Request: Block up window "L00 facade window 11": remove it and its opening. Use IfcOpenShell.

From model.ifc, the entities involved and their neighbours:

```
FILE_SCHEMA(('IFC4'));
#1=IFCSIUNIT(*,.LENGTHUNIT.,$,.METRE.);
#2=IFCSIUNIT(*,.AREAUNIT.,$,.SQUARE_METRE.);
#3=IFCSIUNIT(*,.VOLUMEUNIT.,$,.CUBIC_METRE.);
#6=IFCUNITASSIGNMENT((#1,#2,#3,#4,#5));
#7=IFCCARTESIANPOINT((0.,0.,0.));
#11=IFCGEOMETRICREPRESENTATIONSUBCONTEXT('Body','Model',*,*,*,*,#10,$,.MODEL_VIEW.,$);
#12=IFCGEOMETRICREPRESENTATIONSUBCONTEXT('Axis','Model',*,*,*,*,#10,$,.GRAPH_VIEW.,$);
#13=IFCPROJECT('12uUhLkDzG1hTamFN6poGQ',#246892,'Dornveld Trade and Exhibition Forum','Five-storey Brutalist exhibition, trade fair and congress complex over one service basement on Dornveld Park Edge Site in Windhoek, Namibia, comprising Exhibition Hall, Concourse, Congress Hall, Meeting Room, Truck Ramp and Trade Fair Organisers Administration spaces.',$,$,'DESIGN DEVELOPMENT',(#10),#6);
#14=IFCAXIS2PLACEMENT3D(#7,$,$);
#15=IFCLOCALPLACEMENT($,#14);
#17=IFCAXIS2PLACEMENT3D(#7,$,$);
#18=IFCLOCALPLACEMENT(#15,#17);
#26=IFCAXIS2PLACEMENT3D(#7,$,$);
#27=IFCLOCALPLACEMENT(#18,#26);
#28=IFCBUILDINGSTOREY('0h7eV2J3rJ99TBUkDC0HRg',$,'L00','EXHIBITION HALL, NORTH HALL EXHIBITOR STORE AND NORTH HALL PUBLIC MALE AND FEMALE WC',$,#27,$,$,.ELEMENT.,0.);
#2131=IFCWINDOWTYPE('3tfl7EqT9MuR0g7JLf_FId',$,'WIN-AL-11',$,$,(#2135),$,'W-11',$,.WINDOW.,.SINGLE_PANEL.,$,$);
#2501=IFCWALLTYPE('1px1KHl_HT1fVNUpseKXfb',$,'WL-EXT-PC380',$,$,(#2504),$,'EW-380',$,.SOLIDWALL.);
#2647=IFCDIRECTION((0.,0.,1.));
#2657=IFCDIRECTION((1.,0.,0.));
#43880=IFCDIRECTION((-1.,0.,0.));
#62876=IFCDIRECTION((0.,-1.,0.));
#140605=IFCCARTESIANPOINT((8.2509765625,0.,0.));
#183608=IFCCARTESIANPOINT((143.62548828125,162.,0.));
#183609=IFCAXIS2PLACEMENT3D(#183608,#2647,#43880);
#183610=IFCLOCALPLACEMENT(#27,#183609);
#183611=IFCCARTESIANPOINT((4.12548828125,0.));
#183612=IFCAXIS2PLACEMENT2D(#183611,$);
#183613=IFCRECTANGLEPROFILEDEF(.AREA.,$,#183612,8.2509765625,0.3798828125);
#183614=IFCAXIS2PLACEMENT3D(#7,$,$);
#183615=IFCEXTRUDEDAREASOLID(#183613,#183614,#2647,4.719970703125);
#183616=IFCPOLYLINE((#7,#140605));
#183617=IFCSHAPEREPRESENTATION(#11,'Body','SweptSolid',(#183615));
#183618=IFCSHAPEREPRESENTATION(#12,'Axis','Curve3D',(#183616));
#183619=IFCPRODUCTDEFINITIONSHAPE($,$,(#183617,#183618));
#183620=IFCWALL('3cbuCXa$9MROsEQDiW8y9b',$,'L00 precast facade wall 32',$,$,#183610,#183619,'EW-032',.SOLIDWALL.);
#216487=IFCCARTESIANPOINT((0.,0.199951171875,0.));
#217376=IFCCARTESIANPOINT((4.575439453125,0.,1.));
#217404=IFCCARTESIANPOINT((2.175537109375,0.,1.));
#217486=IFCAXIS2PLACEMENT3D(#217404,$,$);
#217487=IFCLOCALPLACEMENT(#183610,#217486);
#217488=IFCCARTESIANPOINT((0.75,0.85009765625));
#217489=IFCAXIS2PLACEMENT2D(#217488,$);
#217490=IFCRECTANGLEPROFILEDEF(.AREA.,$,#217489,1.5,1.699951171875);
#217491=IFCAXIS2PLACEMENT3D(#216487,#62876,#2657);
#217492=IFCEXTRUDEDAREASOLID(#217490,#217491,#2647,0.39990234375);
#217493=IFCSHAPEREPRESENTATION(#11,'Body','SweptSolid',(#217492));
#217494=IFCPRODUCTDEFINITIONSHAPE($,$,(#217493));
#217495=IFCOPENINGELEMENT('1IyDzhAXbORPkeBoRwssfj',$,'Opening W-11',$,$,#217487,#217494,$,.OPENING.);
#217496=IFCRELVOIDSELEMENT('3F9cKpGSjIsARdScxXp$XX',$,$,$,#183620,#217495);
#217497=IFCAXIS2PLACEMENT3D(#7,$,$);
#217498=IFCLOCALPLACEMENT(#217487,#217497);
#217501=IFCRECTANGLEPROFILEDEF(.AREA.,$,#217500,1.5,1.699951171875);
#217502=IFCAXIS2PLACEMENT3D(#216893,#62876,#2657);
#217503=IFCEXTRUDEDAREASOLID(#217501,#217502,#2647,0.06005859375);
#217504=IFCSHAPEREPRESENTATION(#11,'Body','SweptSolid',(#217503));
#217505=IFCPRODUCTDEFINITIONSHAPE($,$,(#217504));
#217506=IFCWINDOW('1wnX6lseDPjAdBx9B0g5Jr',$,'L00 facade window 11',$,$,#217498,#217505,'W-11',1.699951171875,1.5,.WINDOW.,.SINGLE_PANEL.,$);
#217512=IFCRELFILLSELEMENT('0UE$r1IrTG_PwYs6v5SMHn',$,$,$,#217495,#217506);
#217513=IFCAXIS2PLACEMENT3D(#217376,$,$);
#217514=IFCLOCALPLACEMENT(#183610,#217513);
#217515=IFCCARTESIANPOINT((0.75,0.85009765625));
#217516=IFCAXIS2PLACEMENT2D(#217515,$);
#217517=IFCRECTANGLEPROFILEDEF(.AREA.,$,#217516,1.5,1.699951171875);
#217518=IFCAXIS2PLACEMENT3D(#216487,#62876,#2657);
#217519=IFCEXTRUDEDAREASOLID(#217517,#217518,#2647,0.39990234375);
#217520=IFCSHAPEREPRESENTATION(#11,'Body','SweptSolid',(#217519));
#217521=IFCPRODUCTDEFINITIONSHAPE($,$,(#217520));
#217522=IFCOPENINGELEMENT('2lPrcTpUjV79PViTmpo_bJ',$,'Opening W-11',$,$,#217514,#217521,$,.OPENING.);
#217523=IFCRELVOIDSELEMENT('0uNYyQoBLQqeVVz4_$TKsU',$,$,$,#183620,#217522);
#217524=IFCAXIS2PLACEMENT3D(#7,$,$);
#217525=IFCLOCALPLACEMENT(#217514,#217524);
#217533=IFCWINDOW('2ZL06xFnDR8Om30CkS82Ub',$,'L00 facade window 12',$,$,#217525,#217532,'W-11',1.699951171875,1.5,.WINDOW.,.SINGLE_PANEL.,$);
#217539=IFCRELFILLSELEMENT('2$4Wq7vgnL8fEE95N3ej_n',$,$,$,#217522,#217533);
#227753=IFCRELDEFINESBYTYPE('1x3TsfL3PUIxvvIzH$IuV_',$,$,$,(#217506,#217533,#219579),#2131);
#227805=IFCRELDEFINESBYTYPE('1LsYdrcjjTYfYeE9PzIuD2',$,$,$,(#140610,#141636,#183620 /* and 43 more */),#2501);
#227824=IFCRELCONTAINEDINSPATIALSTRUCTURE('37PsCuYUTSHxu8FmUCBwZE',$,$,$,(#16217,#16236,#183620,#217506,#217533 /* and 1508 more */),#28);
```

```python
import ifcopenshell
import ifcopenshell.api.feature
import ifcopenshell.api.root
import ifcopenshell.geom
import ifcopenshell.util.shape

model = ifcopenshell.open("model.ifc")
settings = ifcopenshell.geom.settings()


def volume(element):
    """Net volume in cubic metres, openings subtracted."""
    shape = ifcopenshell.geom.create_shape(settings, element)
    return ifcopenshell.util.shape.get_volume(shape.geometry)


window = model.by_id(217506)
opening = window.FillsVoids[0].RelatingOpeningElement
wall = opening.VoidsElements[0].RelatingBuildingElement
before = volume(wall)

ifcopenshell.api.root.remove_product(model, product=window)
ifcopenshell.api.feature.remove_feature(model, feature=opening)

after = volume(wall)

print(f"wall volume {before:.3f} -> {after:.3f} m3")

model.write("model_rev.ifc")
```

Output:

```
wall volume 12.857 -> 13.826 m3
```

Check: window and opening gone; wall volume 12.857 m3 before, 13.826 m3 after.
